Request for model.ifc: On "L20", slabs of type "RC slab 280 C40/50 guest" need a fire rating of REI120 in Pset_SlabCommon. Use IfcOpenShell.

First a look at what the model holds.

```python
import ifcopenshell
import ifcopenshell.util.element

model = ifcopenshell.open("model.ifc")
print(model.schema)
storey = next(s for s in model.by_type("IfcBuildingStorey") if s.Name == "L20")
slabs = [e for e in ifcopenshell.util.element.get_decomposition(storey) if e.is_a("IfcSlab")]
seen = {}
for e in slabs:
    element_type = ifcopenshell.util.element.get_type(e)
    key = (element_type.Name if element_type != e and element_type else None, ifcopenshell.util.element.get_pset(e, "Pset_SlabCommon", "FireRating"))
    seen[key] = seen.get(key, 0) + 1
for (name, value), count in sorted(seen.items(), key=str):
    print(count, "x", name, "|", value)
```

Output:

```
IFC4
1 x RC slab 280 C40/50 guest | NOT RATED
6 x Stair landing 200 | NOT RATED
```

```python
import ifcopenshell
import ifcopenshell.api.pset
import ifcopenshell.util.element

model = ifcopenshell.open("model.ifc")

storey = next(s for s in model.by_type("IfcBuildingStorey") if s.Name == "L20")
slabs = [e for e in ifcopenshell.util.element.get_decomposition(storey) if e.is_a("IfcSlab")]

count = 0
for e in slabs:
    element_type = ifcopenshell.util.element.get_type(e)
    if element_type in (None, e) or element_type.Name != "RC slab 280 C40/50 guest":
        continue
    # add_pset returns the element's existing set when there is one.
    pset = ifcopenshell.api.pset.add_pset(model, product=e, name="Pset_SlabCommon")
    ifcopenshell.api.pset.edit_pset(model, pset=pset, properties={"FireRating": "REI120"})
    count += 1

print(count, "slabs updated")

model.write("model_v2.ifc")
```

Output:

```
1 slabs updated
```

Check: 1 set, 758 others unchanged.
